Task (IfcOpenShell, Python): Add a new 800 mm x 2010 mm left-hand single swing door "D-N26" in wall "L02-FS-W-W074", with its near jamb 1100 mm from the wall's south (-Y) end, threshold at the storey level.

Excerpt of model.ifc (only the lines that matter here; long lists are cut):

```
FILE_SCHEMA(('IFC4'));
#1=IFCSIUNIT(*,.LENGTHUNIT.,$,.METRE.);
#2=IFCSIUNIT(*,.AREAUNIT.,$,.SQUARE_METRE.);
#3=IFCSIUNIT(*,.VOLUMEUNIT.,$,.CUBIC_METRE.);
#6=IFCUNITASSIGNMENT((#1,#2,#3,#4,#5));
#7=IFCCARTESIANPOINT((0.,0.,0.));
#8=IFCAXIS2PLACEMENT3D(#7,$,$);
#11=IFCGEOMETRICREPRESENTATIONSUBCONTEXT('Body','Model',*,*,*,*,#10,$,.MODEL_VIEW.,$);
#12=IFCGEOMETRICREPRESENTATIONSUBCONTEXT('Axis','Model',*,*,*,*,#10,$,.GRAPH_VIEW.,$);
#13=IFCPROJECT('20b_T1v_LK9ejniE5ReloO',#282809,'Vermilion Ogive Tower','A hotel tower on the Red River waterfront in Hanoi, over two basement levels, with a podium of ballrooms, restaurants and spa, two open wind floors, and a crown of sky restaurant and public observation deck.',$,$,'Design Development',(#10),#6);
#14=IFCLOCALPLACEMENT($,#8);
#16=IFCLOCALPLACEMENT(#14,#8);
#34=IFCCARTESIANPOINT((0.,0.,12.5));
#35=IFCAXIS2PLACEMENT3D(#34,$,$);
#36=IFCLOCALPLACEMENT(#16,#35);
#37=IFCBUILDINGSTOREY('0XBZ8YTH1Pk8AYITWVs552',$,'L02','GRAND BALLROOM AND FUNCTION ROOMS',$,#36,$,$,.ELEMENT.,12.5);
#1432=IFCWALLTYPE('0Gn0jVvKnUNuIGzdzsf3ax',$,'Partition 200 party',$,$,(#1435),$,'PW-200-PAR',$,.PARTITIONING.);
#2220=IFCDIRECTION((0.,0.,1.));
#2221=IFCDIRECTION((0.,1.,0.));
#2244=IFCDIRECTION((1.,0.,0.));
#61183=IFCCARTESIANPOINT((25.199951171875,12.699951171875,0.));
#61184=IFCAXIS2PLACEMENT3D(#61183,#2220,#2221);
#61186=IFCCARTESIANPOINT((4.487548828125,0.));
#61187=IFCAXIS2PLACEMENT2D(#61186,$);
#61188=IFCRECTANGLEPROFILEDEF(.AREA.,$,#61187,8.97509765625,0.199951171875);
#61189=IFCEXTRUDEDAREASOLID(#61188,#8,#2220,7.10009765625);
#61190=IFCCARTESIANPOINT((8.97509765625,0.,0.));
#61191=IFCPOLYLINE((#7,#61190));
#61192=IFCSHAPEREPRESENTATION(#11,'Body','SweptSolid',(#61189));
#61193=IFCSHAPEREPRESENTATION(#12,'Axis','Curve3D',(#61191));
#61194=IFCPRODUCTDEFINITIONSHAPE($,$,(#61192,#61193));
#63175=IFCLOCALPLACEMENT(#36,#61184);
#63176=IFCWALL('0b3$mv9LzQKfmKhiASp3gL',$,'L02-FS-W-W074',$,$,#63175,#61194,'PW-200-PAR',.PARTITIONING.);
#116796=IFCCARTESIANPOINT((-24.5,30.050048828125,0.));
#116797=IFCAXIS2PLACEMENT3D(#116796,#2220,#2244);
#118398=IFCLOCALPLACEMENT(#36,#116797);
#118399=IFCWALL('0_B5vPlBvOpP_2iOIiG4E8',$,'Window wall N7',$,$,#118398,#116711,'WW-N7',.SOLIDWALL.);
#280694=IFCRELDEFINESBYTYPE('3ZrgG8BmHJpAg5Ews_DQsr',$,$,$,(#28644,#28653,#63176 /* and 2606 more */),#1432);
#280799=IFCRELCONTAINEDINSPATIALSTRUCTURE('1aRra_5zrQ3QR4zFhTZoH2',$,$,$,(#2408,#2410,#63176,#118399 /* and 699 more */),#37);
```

```python
import numpy as np
import ifcopenshell
import ifcopenshell.api.feature
import ifcopenshell.api.geometry
import ifcopenshell.api.root
import ifcopenshell.api.spatial
import ifcopenshell.geom
import ifcopenshell.util.element
import ifcopenshell.util.placement
import ifcopenshell.util.representation
import ifcopenshell.util.shape
import ifcopenshell.util.unit

model = ifcopenshell.open("model.ifc")
unit_scale = ifcopenshell.util.unit.calculate_unit_scale(model)
settings = ifcopenshell.geom.settings()


def volume(element):
    """Net volume in cubic metres, openings subtracted."""
    shape = ifcopenshell.geom.create_shape(settings, element)
    return ifcopenshell.util.shape.get_volume(shape.geometry)


wall = model.by_guid("0b3$mv9LzQKfmKhiASp3gL")
storey = ifcopenshell.util.element.get_container(wall, ifc_class="IfcBuildingStorey")
context = ifcopenshell.util.representation.get_context(model, "Model", "Body", "MODEL_VIEW")
before = volume(wall)

width, height, from_end, sill = 0.8, 2.01, 1.1, 0.0  # metres

# The wall runs along its own X axis, and the end named is its -X end.
wall_shape = ifcopenshell.geom.create_shape(settings, wall)
x, y, z = ifcopenshell.util.shape.get_vertices(wall_shape.geometry).T
start = x.min() + from_end
face, thickness = float(y.min()), float(y.max() - y.min())
wall_matrix = ifcopenshell.util.placement.get_local_placement(wall.ObjectPlacement)
level = ifcopenshell.util.placement.get_local_placement(storey.ObjectPlacement)[2, 3]


def in_wall(x, y):
    """Placement at x, y metres in the wall's axes, at sill height."""
    matrix = wall_matrix.copy()
    matrix[:, 3] = wall_matrix @ np.array([x / unit_scale, y / unit_scale, 0.0, 1.0])
    matrix[2, 3] = level + sill / unit_scale
    return matrix


# Opening: a box that overshoots both wall faces by 50 mm.
opening = ifcopenshell.api.root.create_entity(model, ifc_class="IfcOpeningElement", predefined_type="OPENING")
box = ifcopenshell.api.geometry.add_wall_representation(
    model, context=context, length=width, height=height, thickness=thickness + 0.1
)
ifcopenshell.api.geometry.assign_representation(model, product=opening, representation=box)
ifcopenshell.api.geometry.edit_object_placement(model, product=opening, matrix=in_wall(start, face - 0.05), is_si=False)
ifcopenshell.api.feature.add_feature(model, feature=opening, element=wall)

door = ifcopenshell.api.root.create_entity(model, ifc_class="IfcDoor", name="D-N26", predefined_type="DOOR")
door.OverallWidth, door.OverallHeight = width / unit_scale, height / unit_scale
door.OperationType = "SINGLE_SWING_LEFT"
body = ifcopenshell.api.geometry.add_door_representation(
    model,
    context=context,
    overall_width=door.OverallWidth,
    overall_height=door.OverallHeight,
    operation_type="SINGLE_SWING_LEFT",
    lining_properties={"LiningDepth": thickness / unit_scale, "ThresholdDepth": thickness / unit_scale},
)
ifcopenshell.api.geometry.assign_representation(model, product=door, representation=body)
ifcopenshell.api.spatial.assign_container(model, products=[door], relating_structure=storey)
ifcopenshell.api.feature.add_filling(model, opening=opening, element=door)

# The lining spans the wall, so the door starts at the wall face.
ifcopenshell.api.geometry.edit_object_placement(model, product=door, matrix=in_wall(start, face), is_si=False)

after = volume(wall)

print(f"wall volume {before:.3f} -> {after:.3f} m3")

model.write("model_updated.ifc")
```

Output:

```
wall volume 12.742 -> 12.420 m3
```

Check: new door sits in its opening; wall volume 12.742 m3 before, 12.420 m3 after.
